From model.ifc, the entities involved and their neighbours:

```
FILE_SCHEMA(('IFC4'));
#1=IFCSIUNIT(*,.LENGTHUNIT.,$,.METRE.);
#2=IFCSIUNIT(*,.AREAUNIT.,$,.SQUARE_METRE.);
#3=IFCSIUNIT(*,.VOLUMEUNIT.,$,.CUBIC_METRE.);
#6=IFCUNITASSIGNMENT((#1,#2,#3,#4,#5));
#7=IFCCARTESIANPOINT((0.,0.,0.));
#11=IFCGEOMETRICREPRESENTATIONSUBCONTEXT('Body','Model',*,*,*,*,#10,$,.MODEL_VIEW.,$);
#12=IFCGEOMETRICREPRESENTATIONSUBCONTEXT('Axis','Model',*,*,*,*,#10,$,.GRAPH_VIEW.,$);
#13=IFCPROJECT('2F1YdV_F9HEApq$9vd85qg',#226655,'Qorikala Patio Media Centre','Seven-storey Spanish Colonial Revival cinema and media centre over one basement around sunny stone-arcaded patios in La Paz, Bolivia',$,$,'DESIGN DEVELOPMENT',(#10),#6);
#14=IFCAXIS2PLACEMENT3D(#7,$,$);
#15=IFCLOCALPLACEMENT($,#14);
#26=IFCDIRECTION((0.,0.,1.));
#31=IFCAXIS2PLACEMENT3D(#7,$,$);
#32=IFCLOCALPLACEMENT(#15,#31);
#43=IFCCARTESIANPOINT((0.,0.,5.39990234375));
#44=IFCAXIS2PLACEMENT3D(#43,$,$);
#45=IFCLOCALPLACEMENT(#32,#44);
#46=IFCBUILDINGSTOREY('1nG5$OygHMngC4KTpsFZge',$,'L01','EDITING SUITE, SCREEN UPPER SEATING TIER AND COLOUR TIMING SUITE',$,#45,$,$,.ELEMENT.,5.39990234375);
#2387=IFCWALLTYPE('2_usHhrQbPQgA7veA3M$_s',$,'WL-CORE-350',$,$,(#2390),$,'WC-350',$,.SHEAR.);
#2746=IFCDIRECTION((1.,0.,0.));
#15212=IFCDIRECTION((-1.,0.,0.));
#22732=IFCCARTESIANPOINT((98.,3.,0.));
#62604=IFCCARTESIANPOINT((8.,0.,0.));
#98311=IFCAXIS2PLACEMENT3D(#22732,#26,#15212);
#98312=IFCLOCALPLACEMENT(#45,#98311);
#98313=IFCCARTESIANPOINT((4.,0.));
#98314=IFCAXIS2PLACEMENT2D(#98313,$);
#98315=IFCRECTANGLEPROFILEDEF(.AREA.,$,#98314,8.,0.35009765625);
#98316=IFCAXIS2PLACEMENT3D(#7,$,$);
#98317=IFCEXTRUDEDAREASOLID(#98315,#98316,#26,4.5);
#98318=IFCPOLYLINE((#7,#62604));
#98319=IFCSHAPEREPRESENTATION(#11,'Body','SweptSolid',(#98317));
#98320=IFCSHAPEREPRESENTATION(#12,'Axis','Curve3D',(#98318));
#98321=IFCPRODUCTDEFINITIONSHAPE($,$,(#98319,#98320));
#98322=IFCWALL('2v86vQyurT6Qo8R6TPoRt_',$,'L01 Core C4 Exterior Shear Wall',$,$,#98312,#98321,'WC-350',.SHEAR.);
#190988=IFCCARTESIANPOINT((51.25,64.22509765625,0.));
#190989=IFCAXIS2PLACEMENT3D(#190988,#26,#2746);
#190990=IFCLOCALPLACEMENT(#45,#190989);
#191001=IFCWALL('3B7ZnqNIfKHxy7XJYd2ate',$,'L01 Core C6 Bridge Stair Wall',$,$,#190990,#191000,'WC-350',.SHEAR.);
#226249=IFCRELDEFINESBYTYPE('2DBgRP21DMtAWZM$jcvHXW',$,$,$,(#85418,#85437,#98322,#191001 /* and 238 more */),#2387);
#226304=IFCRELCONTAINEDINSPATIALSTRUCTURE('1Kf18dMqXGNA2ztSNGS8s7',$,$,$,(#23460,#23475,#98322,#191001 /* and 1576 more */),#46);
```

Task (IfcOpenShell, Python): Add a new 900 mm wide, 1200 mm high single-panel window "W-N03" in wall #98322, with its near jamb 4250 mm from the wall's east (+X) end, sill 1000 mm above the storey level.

```python
import numpy as np
import ifcopenshell
import ifcopenshell.api.feature
import ifcopenshell.api.geometry
import ifcopenshell.api.root
import ifcopenshell.api.spatial
import ifcopenshell.geom
import ifcopenshell.util.element
import ifcopenshell.util.placement
import ifcopenshell.util.representation
import ifcopenshell.util.shape
import ifcopenshell.util.unit

model = ifcopenshell.open("model.ifc")
unit_scale = ifcopenshell.util.unit.calculate_unit_scale(model)
settings = ifcopenshell.geom.settings()


def volume(element):
    """Net volume in cubic metres, openings subtracted."""
    shape = ifcopenshell.geom.create_shape(settings, element)
    return ifcopenshell.util.shape.get_volume(shape.geometry)


wall = model.by_guid("2v86vQyurT6Qo8R6TPoRt_")
storey = ifcopenshell.util.element.get_container(wall, ifc_class="IfcBuildingStorey")
context = ifcopenshell.util.representation.get_context(model, "Model", "Body", "MODEL_VIEW")
before = volume(wall)

width, height, from_end, sill = 0.9, 1.2, 4.25, 1  # metres

# The wall runs along its own X axis, and the end named is its -X end.
wall_shape = ifcopenshell.geom.create_shape(settings, wall)
x, y, z = ifcopenshell.util.shape.get_vertices(wall_shape.geometry).T
start = x.min() + from_end
face, thickness = float(y.min()), float(y.max() - y.min())
wall_matrix = ifcopenshell.util.placement.get_local_placement(wall.ObjectPlacement)
level = ifcopenshell.util.placement.get_local_placement(storey.ObjectPlacement)[2, 3]


def in_wall(x, y):
    """Placement at x, y metres in the wall's axes, at sill height."""
    matrix = wall_matrix.copy()
    matrix[:, 3] = wall_matrix @ np.array([x / unit_scale, y / unit_scale, 0.0, 1.0])
    matrix[2, 3] = level + sill / unit_scale
    return matrix


# Opening: a box that overshoots both wall faces by 50 mm.
opening = ifcopenshell.api.root.create_entity(model, ifc_class="IfcOpeningElement", predefined_type="OPENING")
box = ifcopenshell.api.geometry.add_wall_representation(
    model, context=context, length=width, height=height, thickness=thickness + 0.1
)
ifcopenshell.api.geometry.assign_representation(model, product=opening, representation=box)
ifcopenshell.api.geometry.edit_object_placement(model, product=opening, matrix=in_wall(start, face - 0.05), is_si=False)
ifcopenshell.api.feature.add_feature(model, feature=opening, element=wall)

window = ifcopenshell.api.root.create_entity(model, ifc_class="IfcWindow", name="W-N03", predefined_type="WINDOW")
window.OverallWidth, window.OverallHeight = width / unit_scale, height / unit_scale
window.PartitioningType = "SINGLE_PANEL"
body = ifcopenshell.api.geometry.add_window_representation(
    model,
    context=context,
    overall_width=window.OverallWidth,
    overall_height=window.OverallHeight,
    partition_type="SINGLE_PANEL",
)
ifcopenshell.api.geometry.assign_representation(model, product=window, representation=body)
ifcopenshell.api.spatial.assign_container(model, products=[window], relating_structure=storey)
ifcopenshell.api.feature.add_filling(model, opening=opening, element=window)

# Centre the window in the wall's thickness.
ifcopenshell.api.geometry.edit_object_placement(model, product=window, matrix=in_wall(start, face), is_si=False)
window_shape = ifcopenshell.geom.create_shape(settings, window)
depth = ifcopenshell.util.shape.get_vertices(window_shape.geometry)[:, 1]
offset = face + thickness / 2 - (depth.min() + depth.max()) / 2
ifcopenshell.api.geometry.edit_object_placement(model, product=window, matrix=in_wall(start, offset), is_si=False)

after = volume(wall)

print(f"wall volume {before:.3f} -> {after:.3f} m3")

model.write("model-out.ifc")
```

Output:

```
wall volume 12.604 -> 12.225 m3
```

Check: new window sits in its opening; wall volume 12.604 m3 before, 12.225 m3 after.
